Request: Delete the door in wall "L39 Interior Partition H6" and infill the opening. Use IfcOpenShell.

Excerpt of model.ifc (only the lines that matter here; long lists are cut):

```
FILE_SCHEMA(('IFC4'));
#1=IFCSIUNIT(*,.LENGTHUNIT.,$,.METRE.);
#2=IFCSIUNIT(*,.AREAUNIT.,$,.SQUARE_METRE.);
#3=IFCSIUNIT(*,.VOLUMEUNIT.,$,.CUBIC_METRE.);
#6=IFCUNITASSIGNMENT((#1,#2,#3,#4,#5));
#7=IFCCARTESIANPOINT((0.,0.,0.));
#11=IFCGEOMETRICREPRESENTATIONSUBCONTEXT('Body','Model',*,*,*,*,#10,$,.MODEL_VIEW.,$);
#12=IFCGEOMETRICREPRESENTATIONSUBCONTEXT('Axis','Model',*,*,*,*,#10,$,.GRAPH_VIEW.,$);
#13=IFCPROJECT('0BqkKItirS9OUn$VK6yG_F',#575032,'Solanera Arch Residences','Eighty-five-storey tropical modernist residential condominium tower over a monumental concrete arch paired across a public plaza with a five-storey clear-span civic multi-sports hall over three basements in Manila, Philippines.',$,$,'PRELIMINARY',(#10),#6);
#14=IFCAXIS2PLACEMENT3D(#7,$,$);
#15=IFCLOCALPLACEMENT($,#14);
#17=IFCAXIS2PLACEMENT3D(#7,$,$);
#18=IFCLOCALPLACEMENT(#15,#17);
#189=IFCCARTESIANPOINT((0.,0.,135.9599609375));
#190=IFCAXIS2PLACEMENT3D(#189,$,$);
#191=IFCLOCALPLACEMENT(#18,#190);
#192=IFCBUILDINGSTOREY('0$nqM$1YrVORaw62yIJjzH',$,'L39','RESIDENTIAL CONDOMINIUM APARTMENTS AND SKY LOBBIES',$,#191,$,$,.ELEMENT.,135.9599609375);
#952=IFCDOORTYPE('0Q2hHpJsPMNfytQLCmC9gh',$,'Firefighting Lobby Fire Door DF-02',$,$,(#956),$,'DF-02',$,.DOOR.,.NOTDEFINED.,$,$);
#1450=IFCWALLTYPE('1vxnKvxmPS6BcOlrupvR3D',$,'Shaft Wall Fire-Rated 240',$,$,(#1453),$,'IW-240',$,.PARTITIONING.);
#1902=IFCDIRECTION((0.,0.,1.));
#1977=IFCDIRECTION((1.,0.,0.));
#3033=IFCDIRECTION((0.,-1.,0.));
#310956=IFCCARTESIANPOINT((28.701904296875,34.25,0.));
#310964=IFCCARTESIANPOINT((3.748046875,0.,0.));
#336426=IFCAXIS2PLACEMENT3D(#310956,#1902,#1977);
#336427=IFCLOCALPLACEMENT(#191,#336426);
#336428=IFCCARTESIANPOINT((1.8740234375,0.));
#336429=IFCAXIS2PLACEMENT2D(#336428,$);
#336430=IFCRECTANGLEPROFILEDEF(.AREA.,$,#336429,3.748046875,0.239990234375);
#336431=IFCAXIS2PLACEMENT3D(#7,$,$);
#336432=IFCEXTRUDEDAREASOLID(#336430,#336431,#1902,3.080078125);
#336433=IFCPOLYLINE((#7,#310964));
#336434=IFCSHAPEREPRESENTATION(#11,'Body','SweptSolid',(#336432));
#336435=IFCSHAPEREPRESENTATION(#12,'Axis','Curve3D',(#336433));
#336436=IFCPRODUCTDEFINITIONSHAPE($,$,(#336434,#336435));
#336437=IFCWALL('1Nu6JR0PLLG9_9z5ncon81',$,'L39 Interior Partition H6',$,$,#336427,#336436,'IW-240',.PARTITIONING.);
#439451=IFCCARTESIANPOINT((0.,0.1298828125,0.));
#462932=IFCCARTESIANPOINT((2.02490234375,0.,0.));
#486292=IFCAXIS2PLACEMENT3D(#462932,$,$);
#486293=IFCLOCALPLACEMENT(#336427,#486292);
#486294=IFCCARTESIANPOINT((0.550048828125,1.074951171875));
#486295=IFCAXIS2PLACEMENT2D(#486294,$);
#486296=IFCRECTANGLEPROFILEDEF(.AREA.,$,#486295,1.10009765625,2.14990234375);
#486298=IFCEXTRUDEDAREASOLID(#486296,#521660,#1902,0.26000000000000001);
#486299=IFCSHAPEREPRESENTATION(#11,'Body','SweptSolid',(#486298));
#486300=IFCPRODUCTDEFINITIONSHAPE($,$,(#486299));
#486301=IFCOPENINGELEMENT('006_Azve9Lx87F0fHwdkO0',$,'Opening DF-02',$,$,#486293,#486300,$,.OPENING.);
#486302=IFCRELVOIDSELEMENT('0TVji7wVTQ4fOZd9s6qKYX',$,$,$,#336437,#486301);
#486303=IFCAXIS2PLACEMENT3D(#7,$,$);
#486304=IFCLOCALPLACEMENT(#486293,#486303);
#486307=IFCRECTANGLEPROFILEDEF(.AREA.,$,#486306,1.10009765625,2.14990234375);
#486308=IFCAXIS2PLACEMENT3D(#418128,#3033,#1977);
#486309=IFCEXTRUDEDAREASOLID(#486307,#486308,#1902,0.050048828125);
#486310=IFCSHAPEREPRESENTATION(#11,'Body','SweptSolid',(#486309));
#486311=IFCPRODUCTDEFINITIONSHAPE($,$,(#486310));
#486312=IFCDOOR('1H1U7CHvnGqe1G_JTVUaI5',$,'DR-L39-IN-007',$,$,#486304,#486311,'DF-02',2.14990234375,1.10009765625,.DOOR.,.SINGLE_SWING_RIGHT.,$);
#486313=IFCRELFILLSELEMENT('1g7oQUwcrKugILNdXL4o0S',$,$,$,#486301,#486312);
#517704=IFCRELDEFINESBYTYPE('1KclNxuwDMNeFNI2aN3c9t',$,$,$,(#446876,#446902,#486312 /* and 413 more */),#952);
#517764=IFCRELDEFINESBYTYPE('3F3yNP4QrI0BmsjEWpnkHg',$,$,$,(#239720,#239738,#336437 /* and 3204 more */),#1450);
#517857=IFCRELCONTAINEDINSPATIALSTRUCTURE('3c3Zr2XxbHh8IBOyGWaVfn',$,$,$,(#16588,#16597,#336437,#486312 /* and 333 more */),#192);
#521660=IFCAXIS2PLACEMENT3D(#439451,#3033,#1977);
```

```python
import ifcopenshell
import ifcopenshell.api.feature
import ifcopenshell.api.root
import ifcopenshell.geom
import ifcopenshell.util.shape

model = ifcopenshell.open("model.ifc")
settings = ifcopenshell.geom.settings()


def volume(element):
    """Net volume in cubic metres, openings subtracted."""
    shape = ifcopenshell.geom.create_shape(settings, element)
    return ifcopenshell.util.shape.get_volume(shape.geometry)


door = model.by_guid("1H1U7CHvnGqe1G_JTVUaI5")
opening = door.FillsVoids[0].RelatingOpeningElement
wall = opening.VoidsElements[0].RelatingBuildingElement
before = volume(wall)

ifcopenshell.api.root.remove_product(model, product=door)
ifcopenshell.api.feature.remove_feature(model, feature=opening)

after = volume(wall)

print(f"wall volume {before:.3f} -> {after:.3f} m3")

model.write("model_rev.ifc")
```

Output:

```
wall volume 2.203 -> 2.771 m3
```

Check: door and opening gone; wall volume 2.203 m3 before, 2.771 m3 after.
